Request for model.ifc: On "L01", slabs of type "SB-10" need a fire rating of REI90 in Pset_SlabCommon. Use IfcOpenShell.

First a look at what the model holds.

```python
import ifcopenshell
import ifcopenshell.util.element

model = ifcopenshell.open("model.ifc")
print(model.schema)
storey = next(s for s in model.by_type("IfcBuildingStorey") if s.Name == "L01")
slabs = [e for e in ifcopenshell.util.element.get_decomposition(storey) if e.is_a("IfcSlab")]
seen = {}
for e in slabs:
    element_type = ifcopenshell.util.element.get_type(e)
    key = (element_type.Name if element_type != e and element_type else None, ifcopenshell.util.element.get_pset(e, "Pset_SlabCommon", "FireRating"))
    seen[key] = seen.get(key, 0) + 1
for (name, value), count in sorted(seen.items(), key=str):
    print(count, "x", name, "|", value)
```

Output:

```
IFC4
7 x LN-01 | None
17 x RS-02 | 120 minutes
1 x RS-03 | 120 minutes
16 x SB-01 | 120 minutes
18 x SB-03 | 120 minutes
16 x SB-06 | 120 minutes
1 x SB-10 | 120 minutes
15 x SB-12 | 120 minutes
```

```python
import ifcopenshell
import ifcopenshell.api.pset
import ifcopenshell.util.element

model = ifcopenshell.open("model.ifc")

storey = next(s for s in model.by_type("IfcBuildingStorey") if s.Name == "L01")
slabs = [e for e in ifcopenshell.util.element.get_decomposition(storey) if e.is_a("IfcSlab")]

count = 0
for e in slabs:
    element_type = ifcopenshell.util.element.get_type(e)
    if element_type in (None, e) or element_type.Name != "SB-10":
        continue
    # add_pset returns the element's existing set when there is one.
    pset = ifcopenshell.api.pset.add_pset(model, product=e, name="Pset_SlabCommon")
    ifcopenshell.api.pset.edit_pset(model, pset=pset, properties={"FireRating": "REI90"})
    count += 1

print(count, "slabs updated")

model.write("model_rev.ifc")
```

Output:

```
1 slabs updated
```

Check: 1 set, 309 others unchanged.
